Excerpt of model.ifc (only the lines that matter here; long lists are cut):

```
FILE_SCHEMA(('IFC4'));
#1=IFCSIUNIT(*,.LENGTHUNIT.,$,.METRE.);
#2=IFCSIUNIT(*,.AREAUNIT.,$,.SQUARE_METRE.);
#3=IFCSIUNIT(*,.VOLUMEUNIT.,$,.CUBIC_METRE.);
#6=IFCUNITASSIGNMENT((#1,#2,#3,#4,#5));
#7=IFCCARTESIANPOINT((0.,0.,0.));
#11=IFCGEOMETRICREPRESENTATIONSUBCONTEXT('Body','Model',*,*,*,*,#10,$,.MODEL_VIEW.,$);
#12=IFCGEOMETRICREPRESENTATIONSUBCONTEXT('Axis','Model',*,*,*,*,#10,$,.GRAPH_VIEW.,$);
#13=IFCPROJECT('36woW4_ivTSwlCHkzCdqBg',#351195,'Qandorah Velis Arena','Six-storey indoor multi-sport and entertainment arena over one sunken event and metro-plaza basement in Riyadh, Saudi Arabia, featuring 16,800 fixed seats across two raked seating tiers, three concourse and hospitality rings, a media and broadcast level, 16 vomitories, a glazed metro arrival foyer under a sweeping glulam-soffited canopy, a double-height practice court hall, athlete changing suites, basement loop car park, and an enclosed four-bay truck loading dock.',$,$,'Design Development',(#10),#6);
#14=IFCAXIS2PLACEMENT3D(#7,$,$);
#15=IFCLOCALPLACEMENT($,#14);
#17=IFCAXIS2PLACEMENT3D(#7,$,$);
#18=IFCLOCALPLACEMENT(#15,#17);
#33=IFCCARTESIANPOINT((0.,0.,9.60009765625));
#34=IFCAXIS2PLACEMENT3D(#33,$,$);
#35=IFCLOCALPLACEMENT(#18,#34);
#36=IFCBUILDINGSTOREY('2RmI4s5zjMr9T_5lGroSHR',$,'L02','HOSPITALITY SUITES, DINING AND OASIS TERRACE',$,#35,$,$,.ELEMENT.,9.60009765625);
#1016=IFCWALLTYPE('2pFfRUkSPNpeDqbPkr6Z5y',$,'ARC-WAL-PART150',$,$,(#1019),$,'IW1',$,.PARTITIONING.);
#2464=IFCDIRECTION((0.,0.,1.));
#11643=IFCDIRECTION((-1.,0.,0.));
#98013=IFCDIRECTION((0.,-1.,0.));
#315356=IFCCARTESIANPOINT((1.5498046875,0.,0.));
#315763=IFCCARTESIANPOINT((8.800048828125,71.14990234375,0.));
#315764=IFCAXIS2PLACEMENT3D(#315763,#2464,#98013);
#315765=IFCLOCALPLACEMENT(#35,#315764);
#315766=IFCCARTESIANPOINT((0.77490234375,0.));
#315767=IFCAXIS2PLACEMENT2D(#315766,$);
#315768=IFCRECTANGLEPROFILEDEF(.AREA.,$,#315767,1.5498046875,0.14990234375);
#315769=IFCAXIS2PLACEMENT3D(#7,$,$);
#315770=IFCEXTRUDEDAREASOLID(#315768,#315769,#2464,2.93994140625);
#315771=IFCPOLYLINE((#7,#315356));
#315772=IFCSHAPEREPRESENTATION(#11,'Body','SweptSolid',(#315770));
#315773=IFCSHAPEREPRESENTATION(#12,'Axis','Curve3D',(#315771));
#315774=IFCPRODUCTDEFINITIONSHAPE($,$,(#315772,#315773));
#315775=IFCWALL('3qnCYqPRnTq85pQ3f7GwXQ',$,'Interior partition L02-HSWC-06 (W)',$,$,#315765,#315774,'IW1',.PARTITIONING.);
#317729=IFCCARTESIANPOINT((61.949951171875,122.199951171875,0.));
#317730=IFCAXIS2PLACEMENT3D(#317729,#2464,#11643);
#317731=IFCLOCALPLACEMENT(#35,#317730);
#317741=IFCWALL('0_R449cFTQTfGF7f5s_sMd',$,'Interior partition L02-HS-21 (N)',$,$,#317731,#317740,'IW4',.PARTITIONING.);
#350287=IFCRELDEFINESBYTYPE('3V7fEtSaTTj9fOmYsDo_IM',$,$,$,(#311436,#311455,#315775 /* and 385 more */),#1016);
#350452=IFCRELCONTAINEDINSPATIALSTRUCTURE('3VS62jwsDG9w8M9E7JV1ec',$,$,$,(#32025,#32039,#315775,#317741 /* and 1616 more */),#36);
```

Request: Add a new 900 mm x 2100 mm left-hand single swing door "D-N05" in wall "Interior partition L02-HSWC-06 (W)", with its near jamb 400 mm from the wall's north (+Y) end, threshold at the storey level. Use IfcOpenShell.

```python
import numpy as np
import ifcopenshell
import ifcopenshell.api.feature
import ifcopenshell.api.geometry
import ifcopenshell.api.root
import ifcopenshell.api.spatial
import ifcopenshell.geom
import ifcopenshell.util.element
import ifcopenshell.util.placement
import ifcopenshell.util.representation
import ifcopenshell.util.shape
import ifcopenshell.util.unit

model = ifcopenshell.open("model.ifc")
unit_scale = ifcopenshell.util.unit.calculate_unit_scale(model)
settings = ifcopenshell.geom.settings()


def volume(element):
    """Net volume in cubic metres, openings subtracted."""
    shape = ifcopenshell.geom.create_shape(settings, element)
    return ifcopenshell.util.shape.get_volume(shape.geometry)


wall = model.by_id(315775)
storey = ifcopenshell.util.element.get_container(wall, ifc_class="IfcBuildingStorey")
context = ifcopenshell.util.representation.get_context(model, "Model", "Body", "MODEL_VIEW")
before = volume(wall)

width, height, from_end, sill = 0.9, 2.1, 0.4, 0.0  # metres

# The wall runs along its own X axis, and the end named is its -X end.
wall_shape = ifcopenshell.geom.create_shape(settings, wall)
x, y, z = ifcopenshell.util.shape.get_vertices(wall_shape.geometry).T
start = x.min() + from_end
face, thickness = float(y.min()), float(y.max() - y.min())
wall_matrix = ifcopenshell.util.placement.get_local_placement(wall.ObjectPlacement)
level = ifcopenshell.util.placement.get_local_placement(storey.ObjectPlacement)[2, 3]


def in_wall(x, y):
    """Placement at x, y metres in the wall's axes, at sill height."""
    matrix = wall_matrix.copy()
    matrix[:, 3] = wall_matrix @ np.array([x / unit_scale, y / unit_scale, 0.0, 1.0])
    matrix[2, 3] = level + sill / unit_scale
    return matrix


# Opening: a box that overshoots both wall faces by 50 mm.
opening = ifcopenshell.api.root.create_entity(model, ifc_class="IfcOpeningElement", predefined_type="OPENING")
box = ifcopenshell.api.geometry.add_wall_representation(
    model, context=context, length=width, height=height, thickness=thickness + 0.1
)
ifcopenshell.api.geometry.assign_representation(model, product=opening, representation=box)
ifcopenshell.api.geometry.edit_object_placement(model, product=opening, matrix=in_wall(start, face - 0.05), is_si=False)
ifcopenshell.api.feature.add_feature(model, feature=opening, element=wall)

door = ifcopenshell.api.root.create_entity(model, ifc_class="IfcDoor", name="D-N05", predefined_type="DOOR")
door.OverallWidth, door.OverallHeight = width / unit_scale, height / unit_scale
door.OperationType = "SINGLE_SWING_LEFT"
body = ifcopenshell.api.geometry.add_door_representation(
    model,
    context=context,
    overall_width=door.OverallWidth,
    overall_height=door.OverallHeight,
    operation_type="SINGLE_SWING_LEFT",
    lining_properties={"LiningDepth": thickness / unit_scale, "ThresholdDepth": thickness / unit_scale},
)
ifcopenshell.api.geometry.assign_representation(model, product=door, representation=body)
ifcopenshell.api.spatial.assign_container(model, products=[door], relating_structure=storey)
ifcopenshell.api.feature.add_filling(model, opening=opening, element=door)

# The lining spans the wall, so the door starts at the wall face.
ifcopenshell.api.geometry.edit_object_placement(model, product=door, matrix=in_wall(start, face), is_si=False)

after = volume(wall)

print(f"wall volume {before:.3f} -> {after:.3f} m3")

model.write("model-out.ifc")
```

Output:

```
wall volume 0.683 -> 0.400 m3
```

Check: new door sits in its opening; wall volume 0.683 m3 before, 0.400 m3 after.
